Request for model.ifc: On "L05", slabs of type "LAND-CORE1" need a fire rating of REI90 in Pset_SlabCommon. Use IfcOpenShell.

First a look at what the model holds.

```python
import ifcopenshell
import ifcopenshell.util.element

model = ifcopenshell.open("model.ifc")
print(model.schema)
storey = next(s for s in model.by_type("IfcBuildingStorey") if s.Name == "L05")
slabs = [e for e in ifcopenshell.util.element.get_decomposition(storey) if e.is_a("IfcSlab")]
seen = {}
for e in slabs:
    element_type = ifcopenshell.util.element.get_type(e)
    key = (element_type.Name if element_type != e and element_type else None, ifcopenshell.util.element.get_pset(e, "Pset_SlabCommon", "FireRating"))
    seen[key] = seen.get(key, 0) + 1
for (name, value), count in sorted(seen.items(), key=str):
    print(count, "x", name, "|", value)
```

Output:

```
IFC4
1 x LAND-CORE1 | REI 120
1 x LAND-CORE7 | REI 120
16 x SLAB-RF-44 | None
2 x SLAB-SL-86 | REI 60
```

```python
import ifcopenshell
import ifcopenshell.api.pset
import ifcopenshell.util.element

model = ifcopenshell.open("model.ifc")

storey = next(s for s in model.by_type("IfcBuildingStorey") if s.Name == "L05")
slabs = [e for e in ifcopenshell.util.element.get_decomposition(storey) if e.is_a("IfcSlab")]

count = 0
for e in slabs:
    element_type = ifcopenshell.util.element.get_type(e)
    if element_type in (None, e) or element_type.Name != "LAND-CORE1":
        continue
    # add_pset returns the element's existing set when there is one.
    pset = ifcopenshell.api.pset.add_pset(model, product=e, name="Pset_SlabCommon")
    ifcopenshell.api.pset.edit_pset(model, pset=pset, properties={"FireRating": "REI90"})
    count += 1

print(count, "slabs updated")

model.write("model_edited.ifc")
```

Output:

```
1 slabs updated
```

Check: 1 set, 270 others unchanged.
